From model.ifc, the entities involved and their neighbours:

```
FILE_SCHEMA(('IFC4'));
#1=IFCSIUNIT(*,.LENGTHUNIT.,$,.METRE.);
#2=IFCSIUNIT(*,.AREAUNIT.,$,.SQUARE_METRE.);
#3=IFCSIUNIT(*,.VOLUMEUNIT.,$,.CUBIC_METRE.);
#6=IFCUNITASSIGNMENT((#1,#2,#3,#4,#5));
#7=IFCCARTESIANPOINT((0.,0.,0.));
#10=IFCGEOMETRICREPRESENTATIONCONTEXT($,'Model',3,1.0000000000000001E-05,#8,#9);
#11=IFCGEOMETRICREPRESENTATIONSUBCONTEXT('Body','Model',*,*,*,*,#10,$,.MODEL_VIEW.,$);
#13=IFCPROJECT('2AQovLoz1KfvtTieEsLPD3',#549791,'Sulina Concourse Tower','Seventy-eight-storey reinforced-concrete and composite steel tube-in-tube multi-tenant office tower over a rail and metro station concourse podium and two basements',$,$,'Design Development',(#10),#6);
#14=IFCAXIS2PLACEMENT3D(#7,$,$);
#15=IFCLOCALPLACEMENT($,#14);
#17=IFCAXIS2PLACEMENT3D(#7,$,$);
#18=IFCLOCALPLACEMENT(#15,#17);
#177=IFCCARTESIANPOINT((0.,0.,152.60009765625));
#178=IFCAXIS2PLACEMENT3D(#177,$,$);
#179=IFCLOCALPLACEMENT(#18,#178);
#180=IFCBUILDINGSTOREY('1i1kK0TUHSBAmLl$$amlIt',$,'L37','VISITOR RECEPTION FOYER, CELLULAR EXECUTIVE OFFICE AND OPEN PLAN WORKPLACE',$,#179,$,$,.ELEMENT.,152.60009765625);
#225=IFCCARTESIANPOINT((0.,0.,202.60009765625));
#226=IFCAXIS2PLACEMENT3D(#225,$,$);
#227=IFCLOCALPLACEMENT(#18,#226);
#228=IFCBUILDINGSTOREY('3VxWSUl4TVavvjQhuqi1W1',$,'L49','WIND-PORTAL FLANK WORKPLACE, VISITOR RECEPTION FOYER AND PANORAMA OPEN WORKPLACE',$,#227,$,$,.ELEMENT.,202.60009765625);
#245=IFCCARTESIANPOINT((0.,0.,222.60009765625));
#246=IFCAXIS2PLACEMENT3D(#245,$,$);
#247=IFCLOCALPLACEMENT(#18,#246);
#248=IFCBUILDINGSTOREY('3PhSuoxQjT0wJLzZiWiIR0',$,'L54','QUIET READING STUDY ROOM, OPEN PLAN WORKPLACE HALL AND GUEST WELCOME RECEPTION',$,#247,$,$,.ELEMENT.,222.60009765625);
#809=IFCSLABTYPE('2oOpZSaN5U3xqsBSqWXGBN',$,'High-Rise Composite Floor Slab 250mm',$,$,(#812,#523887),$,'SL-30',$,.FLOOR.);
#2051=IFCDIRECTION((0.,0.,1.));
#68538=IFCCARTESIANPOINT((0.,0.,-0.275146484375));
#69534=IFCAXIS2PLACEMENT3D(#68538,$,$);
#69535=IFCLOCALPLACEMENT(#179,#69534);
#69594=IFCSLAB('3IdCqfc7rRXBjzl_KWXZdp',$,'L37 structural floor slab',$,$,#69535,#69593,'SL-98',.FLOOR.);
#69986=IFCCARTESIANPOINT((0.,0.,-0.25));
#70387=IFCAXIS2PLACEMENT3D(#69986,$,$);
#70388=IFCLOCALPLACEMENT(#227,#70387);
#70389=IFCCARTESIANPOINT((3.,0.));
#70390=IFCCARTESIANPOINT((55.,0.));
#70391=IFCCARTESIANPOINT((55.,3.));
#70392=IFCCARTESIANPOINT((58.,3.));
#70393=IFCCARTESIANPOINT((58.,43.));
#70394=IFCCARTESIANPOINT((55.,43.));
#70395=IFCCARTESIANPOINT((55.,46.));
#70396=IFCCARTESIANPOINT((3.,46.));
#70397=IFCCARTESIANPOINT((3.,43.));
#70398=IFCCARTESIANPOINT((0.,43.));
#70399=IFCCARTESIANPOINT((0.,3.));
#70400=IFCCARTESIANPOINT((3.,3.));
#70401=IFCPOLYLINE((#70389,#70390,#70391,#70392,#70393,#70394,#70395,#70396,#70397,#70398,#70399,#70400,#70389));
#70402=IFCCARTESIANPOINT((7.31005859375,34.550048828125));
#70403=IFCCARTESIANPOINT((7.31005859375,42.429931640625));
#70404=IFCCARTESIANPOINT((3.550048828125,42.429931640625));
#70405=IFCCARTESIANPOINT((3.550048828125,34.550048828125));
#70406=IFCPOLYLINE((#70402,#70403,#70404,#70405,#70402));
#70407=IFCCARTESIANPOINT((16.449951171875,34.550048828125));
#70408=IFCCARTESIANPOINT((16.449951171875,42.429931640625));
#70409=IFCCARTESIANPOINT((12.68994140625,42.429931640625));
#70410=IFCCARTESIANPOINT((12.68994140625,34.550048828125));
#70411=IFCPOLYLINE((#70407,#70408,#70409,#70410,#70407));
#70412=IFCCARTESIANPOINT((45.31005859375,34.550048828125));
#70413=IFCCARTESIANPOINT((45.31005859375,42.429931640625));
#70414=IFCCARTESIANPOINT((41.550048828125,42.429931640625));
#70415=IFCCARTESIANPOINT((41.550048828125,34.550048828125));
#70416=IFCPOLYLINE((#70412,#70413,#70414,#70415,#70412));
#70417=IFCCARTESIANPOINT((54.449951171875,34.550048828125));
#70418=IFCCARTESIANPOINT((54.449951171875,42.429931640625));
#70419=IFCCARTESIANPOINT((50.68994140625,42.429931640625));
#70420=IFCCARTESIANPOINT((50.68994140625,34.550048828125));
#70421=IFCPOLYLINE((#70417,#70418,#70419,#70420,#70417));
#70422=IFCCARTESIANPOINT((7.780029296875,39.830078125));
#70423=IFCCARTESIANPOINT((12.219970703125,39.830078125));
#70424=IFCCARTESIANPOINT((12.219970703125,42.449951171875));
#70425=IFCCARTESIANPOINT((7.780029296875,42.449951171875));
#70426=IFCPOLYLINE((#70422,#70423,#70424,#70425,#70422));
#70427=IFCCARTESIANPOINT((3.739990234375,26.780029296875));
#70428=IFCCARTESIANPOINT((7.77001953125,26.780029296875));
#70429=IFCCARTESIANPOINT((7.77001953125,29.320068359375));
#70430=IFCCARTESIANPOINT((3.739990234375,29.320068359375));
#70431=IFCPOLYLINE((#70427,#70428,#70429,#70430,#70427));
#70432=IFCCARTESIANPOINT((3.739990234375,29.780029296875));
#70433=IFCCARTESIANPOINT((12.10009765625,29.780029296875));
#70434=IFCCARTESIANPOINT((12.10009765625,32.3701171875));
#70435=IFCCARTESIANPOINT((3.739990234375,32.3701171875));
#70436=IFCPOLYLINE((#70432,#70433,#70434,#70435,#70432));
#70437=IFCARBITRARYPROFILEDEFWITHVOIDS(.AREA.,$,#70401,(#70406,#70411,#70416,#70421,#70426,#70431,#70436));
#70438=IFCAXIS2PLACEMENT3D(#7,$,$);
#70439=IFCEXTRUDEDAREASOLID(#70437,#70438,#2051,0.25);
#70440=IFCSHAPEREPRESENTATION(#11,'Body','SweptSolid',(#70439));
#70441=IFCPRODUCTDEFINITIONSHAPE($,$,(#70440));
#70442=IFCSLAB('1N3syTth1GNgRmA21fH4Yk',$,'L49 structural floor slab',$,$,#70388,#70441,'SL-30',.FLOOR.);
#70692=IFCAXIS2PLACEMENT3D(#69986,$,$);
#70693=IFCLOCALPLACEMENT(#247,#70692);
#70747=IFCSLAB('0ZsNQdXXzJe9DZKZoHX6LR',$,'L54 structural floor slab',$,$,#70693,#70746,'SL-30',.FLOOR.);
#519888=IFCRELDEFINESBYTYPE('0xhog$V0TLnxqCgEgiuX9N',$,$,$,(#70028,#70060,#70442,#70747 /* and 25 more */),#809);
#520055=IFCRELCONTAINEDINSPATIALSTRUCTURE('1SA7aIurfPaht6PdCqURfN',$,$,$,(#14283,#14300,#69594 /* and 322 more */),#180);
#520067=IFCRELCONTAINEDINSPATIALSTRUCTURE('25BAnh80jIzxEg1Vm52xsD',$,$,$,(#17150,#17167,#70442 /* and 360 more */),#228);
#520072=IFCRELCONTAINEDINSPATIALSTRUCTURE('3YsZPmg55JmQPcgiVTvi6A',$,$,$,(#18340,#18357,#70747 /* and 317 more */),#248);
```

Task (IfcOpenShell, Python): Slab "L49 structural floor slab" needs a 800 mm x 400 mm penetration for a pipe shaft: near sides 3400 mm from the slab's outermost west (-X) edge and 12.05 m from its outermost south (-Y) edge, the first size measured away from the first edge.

```python
import numpy as np
import ifcopenshell
import ifcopenshell.api.feature
import ifcopenshell.api.geometry
import ifcopenshell.api.root
import ifcopenshell.geom
import ifcopenshell.util.placement
import ifcopenshell.util.representation
import ifcopenshell.util.shape
import ifcopenshell.util.unit

model = ifcopenshell.open("model.ifc")
unit_scale = ifcopenshell.util.unit.calculate_unit_scale(model)
settings = ifcopenshell.geom.settings()


def volume(element):
    """Net volume in cubic metres, openings subtracted."""
    shape = ifcopenshell.geom.create_shape(settings, element)
    return ifcopenshell.util.shape.get_volume(shape.geometry)


slab = model.by_guid("1N3syTth1GNgRmA21fH4Yk")
before = volume(slab)

# Extent in the slab's own axes, in metres. The edges named are its -X and -Y sides.
slab_shape = ifcopenshell.geom.create_shape(settings, slab)
vertices = ifcopenshell.util.shape.get_vertices(slab_shape.geometry)
x_min, y_min, bottom = vertices.min(axis=0)
top = vertices[:, 2].max()

opening = ifcopenshell.api.root.create_entity(model, ifc_class="IfcOpeningElement", name="Pipe shaft opening", predefined_type="OPENING")
context = ifcopenshell.util.representation.get_context(model, "Model", "Body", "MODEL_VIEW")
width, depth = 0.8, 0.4
outline = [(0.0, 0.0), (width, 0.0), (width, depth), (0.0, depth), (0.0, 0.0)]
# Overshoot both faces by 50 mm so the cut is clean.
shape = ifcopenshell.api.geometry.add_slab_representation(
    model, context=context, depth=top - bottom + 0.1, polyline=outline
)
ifcopenshell.api.geometry.assign_representation(model, product=opening, representation=shape)

matrix = ifcopenshell.util.placement.get_local_placement(slab.ObjectPlacement)
matrix[:, 3] = matrix @ np.append(np.array([x_min + 3.4, y_min + 12.05, bottom - 0.05]) / unit_scale, 1.0)
ifcopenshell.api.geometry.edit_object_placement(model, product=opening, matrix=matrix, is_si=False)
ifcopenshell.api.feature.add_feature(model, feature=opening, element=slab)

after = volume(slab)

print(f"slab volume {before:.3f} -> {after:.3f} m3")

model.write("model-out.ifc")
```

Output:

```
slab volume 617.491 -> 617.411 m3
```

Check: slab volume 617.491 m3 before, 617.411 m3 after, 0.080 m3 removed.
